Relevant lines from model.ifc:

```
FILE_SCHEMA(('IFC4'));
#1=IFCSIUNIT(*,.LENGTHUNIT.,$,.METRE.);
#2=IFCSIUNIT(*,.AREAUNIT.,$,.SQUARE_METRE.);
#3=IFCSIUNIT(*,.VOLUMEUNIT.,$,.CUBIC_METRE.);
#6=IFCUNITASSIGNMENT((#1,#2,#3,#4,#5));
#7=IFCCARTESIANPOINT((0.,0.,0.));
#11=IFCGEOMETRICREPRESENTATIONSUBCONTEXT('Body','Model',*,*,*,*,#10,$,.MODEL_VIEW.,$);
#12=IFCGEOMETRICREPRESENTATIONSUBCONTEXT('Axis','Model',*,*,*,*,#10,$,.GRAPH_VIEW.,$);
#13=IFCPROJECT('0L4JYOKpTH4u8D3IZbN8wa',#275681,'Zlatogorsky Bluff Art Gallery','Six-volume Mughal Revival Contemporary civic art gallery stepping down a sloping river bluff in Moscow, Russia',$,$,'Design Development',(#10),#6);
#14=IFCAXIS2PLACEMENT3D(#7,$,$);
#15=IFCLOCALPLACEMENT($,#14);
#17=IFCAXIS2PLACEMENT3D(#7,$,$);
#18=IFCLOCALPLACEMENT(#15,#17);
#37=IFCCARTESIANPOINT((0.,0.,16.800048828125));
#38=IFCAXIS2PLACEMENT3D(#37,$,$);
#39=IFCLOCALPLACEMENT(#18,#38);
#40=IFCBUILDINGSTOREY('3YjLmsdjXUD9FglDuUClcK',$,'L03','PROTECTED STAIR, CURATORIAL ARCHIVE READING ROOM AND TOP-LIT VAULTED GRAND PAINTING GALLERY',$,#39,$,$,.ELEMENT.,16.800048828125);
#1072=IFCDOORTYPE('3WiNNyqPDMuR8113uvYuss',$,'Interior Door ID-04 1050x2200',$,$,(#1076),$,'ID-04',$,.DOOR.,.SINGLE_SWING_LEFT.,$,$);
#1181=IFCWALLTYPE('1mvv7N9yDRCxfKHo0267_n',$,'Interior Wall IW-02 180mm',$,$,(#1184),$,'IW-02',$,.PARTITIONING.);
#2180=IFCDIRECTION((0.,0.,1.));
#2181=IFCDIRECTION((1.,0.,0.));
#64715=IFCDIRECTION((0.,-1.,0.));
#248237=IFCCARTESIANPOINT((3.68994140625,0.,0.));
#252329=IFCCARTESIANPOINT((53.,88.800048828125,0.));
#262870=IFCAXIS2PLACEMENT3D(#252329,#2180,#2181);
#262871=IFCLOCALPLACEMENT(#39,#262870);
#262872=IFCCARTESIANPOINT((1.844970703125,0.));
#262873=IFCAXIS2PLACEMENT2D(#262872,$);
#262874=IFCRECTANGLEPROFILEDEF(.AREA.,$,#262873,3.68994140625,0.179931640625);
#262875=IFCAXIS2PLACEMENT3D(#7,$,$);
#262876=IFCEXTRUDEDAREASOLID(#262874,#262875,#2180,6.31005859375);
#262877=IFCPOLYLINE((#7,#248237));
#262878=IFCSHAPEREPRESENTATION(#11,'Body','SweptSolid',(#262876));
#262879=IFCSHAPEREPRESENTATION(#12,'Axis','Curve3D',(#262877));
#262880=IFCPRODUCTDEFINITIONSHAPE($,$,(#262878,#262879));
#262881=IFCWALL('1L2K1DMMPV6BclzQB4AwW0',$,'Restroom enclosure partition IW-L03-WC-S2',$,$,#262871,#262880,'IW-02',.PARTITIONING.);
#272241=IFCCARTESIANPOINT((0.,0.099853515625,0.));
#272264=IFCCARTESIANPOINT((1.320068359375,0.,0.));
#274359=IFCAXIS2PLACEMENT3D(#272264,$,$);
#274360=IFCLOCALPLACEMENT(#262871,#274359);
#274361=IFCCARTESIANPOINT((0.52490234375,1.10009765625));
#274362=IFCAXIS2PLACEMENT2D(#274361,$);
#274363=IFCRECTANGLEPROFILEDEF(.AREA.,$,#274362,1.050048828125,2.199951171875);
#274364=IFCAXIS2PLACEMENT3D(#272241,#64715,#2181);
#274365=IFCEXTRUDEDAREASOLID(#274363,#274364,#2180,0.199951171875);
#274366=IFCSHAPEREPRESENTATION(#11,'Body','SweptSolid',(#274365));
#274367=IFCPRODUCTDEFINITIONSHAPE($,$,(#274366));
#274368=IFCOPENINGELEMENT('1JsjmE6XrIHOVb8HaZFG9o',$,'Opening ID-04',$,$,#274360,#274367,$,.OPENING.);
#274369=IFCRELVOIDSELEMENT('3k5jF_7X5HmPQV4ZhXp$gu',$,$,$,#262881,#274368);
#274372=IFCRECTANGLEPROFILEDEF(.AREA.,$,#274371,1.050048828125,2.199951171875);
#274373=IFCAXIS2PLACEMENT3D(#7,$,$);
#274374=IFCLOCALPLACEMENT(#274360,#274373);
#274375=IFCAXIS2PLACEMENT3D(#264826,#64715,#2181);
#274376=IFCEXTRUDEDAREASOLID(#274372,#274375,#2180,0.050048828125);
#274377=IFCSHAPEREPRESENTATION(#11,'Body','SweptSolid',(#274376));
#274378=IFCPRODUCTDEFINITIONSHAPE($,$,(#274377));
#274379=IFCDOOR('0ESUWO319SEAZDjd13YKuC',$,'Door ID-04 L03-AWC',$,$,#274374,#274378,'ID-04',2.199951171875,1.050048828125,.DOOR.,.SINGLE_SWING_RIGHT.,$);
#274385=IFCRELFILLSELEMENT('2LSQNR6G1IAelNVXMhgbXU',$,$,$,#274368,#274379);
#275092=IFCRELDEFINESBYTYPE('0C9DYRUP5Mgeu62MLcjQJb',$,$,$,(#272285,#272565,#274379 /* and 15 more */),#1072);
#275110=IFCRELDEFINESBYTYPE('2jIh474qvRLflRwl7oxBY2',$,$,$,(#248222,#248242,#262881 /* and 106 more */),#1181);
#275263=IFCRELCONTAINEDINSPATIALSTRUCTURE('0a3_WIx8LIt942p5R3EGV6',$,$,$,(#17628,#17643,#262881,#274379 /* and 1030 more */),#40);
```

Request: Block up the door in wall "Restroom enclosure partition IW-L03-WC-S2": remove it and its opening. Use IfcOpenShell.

```python
import ifcopenshell
import ifcopenshell.api.feature
import ifcopenshell.api.root
import ifcopenshell.geom
import ifcopenshell.util.shape

model = ifcopenshell.open("model.ifc")
settings = ifcopenshell.geom.settings()


def volume(element):
    """Net volume in cubic metres, openings subtracted."""
    shape = ifcopenshell.geom.create_shape(settings, element)
    return ifcopenshell.util.shape.get_volume(shape.geometry)


door = model.by_guid("0ESUWO319SEAZDjd13YKuC")
opening = door.FillsVoids[0].RelatingOpeningElement
wall = opening.VoidsElements[0].RelatingBuildingElement
before = volume(wall)

ifcopenshell.api.root.remove_product(model, product=door)
ifcopenshell.api.feature.remove_feature(model, feature=opening)

after = volume(wall)

print(f"wall volume {before:.3f} -> {after:.3f} m3")

model.write("model-out.ifc")
```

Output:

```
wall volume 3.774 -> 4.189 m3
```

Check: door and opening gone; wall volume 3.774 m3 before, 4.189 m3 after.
